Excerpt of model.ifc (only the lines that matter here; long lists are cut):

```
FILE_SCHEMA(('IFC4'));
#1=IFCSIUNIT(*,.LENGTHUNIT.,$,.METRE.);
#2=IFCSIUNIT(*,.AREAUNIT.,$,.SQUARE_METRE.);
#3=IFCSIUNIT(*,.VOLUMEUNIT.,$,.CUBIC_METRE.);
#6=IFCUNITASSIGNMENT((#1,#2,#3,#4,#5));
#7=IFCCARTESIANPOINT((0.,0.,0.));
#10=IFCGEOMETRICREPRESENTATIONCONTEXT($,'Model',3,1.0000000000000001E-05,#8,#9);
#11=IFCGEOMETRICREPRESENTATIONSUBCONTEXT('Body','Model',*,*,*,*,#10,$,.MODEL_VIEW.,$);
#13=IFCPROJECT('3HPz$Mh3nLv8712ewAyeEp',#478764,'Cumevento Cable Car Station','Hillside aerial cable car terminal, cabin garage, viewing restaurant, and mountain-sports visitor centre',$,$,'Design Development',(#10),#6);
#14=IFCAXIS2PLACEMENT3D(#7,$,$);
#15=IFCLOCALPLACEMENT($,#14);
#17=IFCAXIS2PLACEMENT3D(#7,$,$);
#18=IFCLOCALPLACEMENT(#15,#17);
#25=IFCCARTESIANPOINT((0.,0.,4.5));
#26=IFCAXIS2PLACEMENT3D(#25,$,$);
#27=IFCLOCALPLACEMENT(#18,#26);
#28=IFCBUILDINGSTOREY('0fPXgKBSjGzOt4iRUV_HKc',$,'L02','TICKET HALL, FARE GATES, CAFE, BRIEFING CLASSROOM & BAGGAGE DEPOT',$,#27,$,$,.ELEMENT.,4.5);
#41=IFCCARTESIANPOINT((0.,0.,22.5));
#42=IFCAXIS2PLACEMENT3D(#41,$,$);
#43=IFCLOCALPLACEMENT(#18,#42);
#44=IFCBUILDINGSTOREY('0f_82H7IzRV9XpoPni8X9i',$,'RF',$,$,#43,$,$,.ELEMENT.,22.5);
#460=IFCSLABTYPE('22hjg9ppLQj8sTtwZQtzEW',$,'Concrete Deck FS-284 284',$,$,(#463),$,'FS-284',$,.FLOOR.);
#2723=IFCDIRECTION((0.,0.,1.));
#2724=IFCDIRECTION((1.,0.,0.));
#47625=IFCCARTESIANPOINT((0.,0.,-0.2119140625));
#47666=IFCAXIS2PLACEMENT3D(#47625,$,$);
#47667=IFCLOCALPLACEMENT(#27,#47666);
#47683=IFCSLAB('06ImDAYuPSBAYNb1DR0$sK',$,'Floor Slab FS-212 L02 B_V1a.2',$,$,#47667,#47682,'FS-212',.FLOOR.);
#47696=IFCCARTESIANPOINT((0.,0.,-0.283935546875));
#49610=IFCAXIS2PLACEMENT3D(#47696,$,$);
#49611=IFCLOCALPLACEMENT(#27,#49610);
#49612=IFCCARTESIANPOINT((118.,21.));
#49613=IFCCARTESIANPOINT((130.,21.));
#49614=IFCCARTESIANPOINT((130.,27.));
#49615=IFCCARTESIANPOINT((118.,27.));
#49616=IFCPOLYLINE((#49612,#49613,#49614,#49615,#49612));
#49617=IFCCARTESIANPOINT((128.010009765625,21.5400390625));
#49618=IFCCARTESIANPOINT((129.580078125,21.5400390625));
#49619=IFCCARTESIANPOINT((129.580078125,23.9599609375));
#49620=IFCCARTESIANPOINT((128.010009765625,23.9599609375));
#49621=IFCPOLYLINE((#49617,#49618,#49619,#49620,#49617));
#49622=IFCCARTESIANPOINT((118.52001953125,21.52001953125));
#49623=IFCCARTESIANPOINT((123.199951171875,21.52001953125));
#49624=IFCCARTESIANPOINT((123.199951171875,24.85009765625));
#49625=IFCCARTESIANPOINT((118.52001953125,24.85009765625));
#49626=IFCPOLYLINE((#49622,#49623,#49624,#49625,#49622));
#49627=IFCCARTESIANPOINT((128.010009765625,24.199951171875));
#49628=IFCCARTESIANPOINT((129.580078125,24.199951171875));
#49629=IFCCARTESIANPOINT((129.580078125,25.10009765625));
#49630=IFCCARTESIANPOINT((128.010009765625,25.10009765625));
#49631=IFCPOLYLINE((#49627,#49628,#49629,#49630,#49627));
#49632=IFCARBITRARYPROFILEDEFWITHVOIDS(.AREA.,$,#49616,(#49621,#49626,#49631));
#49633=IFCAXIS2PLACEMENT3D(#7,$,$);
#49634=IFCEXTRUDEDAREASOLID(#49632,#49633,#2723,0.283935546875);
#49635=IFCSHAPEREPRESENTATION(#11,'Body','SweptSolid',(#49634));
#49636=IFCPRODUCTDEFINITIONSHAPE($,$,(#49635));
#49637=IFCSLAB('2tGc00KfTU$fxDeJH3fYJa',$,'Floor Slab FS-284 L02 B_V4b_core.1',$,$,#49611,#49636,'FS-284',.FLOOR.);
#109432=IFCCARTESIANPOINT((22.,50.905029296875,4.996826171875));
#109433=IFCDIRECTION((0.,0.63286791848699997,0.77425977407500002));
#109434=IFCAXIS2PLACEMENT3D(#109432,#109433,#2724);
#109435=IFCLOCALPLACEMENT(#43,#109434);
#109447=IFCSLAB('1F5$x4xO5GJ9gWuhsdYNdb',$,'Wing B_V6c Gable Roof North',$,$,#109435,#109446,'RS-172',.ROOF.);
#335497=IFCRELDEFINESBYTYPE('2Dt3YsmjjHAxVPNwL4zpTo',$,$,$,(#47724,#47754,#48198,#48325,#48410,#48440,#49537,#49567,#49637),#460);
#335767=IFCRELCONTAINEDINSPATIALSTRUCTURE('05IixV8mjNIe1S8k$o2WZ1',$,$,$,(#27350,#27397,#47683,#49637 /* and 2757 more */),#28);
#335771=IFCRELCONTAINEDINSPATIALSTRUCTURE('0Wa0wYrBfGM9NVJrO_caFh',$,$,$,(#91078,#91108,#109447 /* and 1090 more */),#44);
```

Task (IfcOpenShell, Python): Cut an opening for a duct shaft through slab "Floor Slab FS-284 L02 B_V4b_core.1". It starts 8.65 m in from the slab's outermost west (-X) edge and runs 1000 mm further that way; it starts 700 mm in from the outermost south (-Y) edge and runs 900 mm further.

```python
import numpy as np
import ifcopenshell
import ifcopenshell.api.feature
import ifcopenshell.api.geometry
import ifcopenshell.api.root
import ifcopenshell.geom
import ifcopenshell.util.placement
import ifcopenshell.util.representation
import ifcopenshell.util.shape
import ifcopenshell.util.unit

model = ifcopenshell.open("model.ifc")
unit_scale = ifcopenshell.util.unit.calculate_unit_scale(model)
settings = ifcopenshell.geom.settings()


def volume(element):
    """Net volume in cubic metres, openings subtracted."""
    shape = ifcopenshell.geom.create_shape(settings, element)
    return ifcopenshell.util.shape.get_volume(shape.geometry)


slab = model.by_guid("2tGc00KfTU$fxDeJH3fYJa")
before = volume(slab)

# Extent in the slab's own axes, in metres. The edges named are its -X and -Y sides.
slab_shape = ifcopenshell.geom.create_shape(settings, slab)
vertices = ifcopenshell.util.shape.get_vertices(slab_shape.geometry)
x_min, y_min, bottom = vertices.min(axis=0)
top = vertices[:, 2].max()

opening = ifcopenshell.api.root.create_entity(model, ifc_class="IfcOpeningElement", name="Duct shaft opening", predefined_type="OPENING")
context = ifcopenshell.util.representation.get_context(model, "Model", "Body", "MODEL_VIEW")
width, depth = 1, 0.9
outline = [(0.0, 0.0), (width, 0.0), (width, depth), (0.0, depth), (0.0, 0.0)]
# Overshoot both faces by 50 mm so the cut is clean.
shape = ifcopenshell.api.geometry.add_slab_representation(
    model, context=context, depth=top - bottom + 0.1, polyline=outline
)
ifcopenshell.api.geometry.assign_representation(model, product=opening, representation=shape)

matrix = ifcopenshell.util.placement.get_local_placement(slab.ObjectPlacement)
matrix[:, 3] = matrix @ np.append(np.array([x_min + 8.65, y_min + 0.7, bottom - 0.05]) / unit_scale, 1.0)
ifcopenshell.api.geometry.edit_object_placement(model, product=opening, matrix=matrix, is_si=False)
ifcopenshell.api.feature.add_feature(model, feature=opening, element=slab)

after = volume(slab)

print(f"slab volume {before:.3f} -> {after:.3f} m3")

model.write("model_rev.ifc")
```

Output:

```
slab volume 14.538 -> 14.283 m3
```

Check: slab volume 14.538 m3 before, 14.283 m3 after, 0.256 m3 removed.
